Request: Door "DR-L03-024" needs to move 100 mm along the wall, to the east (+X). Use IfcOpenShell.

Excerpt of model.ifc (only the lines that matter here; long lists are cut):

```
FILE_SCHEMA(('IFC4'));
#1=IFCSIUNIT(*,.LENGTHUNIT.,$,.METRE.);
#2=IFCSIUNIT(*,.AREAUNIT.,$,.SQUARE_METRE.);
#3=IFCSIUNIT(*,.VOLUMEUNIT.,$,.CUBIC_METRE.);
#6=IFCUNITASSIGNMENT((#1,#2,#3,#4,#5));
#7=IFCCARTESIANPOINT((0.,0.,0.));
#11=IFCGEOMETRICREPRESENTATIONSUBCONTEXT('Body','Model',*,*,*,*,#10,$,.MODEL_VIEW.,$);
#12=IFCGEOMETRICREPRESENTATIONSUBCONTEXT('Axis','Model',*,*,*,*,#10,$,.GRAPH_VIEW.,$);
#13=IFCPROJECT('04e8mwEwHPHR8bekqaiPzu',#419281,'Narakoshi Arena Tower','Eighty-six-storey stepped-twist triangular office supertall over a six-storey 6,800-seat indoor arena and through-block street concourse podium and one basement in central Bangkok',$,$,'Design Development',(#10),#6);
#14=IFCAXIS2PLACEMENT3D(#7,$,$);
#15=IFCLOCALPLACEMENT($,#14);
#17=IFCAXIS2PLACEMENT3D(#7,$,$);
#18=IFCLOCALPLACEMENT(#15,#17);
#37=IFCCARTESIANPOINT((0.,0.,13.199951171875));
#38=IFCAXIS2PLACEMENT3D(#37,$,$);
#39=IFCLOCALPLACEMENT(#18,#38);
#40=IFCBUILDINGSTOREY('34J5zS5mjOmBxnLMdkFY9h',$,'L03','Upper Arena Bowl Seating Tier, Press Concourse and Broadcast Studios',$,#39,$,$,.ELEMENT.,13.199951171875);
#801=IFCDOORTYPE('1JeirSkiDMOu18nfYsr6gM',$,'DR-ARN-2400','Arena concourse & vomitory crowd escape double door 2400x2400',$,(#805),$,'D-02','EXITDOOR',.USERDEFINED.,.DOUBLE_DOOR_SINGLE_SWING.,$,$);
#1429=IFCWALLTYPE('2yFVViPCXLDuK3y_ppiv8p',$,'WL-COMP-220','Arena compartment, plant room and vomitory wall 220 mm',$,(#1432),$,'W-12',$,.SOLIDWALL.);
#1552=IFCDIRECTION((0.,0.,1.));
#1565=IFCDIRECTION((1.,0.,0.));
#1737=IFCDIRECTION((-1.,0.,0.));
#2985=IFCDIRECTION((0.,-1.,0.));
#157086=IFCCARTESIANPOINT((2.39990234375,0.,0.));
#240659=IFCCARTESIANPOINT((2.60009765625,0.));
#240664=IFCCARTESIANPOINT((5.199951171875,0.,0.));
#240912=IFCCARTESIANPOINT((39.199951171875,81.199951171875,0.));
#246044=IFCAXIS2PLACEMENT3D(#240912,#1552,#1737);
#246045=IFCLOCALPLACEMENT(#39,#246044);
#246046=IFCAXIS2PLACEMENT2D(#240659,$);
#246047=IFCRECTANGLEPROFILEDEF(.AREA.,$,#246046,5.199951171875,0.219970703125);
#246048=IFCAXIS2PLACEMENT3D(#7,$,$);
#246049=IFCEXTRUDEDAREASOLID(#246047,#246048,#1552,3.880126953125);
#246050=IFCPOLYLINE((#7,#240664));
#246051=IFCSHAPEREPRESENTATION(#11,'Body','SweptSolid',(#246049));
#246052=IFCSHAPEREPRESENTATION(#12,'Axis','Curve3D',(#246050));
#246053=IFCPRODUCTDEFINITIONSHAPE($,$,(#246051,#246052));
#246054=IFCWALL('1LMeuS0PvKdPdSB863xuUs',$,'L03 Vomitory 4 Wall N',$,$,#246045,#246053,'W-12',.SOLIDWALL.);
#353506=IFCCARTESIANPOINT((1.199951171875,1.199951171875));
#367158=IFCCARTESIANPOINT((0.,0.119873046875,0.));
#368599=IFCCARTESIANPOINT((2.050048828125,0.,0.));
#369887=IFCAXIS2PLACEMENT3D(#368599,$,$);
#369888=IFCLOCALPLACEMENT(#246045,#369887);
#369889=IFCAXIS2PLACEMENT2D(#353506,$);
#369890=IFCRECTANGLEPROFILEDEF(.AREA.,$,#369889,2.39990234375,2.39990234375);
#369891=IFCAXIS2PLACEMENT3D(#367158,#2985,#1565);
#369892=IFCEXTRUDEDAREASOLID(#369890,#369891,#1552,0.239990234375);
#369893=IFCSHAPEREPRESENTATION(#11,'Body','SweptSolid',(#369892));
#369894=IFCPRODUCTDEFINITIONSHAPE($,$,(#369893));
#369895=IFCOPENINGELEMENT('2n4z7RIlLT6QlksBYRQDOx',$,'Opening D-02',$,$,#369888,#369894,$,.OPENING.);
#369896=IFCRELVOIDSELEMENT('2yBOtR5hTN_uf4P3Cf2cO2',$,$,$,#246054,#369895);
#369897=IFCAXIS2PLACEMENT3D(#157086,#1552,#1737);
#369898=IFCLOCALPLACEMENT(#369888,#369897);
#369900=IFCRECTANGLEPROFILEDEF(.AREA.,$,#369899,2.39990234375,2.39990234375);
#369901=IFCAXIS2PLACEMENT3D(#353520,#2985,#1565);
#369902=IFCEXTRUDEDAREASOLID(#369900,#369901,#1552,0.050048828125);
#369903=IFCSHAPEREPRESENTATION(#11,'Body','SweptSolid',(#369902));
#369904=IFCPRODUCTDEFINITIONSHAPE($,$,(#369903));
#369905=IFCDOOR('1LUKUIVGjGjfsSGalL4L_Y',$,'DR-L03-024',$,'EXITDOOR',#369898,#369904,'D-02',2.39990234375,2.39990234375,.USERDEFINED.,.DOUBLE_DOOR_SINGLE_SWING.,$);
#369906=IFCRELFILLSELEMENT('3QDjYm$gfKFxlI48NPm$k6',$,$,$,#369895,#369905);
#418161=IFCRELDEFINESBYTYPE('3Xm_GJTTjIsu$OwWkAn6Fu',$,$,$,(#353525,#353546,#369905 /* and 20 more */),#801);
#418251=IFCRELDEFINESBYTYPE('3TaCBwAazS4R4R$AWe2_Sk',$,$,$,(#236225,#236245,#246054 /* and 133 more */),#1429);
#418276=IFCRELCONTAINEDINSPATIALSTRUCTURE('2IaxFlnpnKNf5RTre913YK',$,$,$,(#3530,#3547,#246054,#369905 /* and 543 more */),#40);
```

```python
import ifcopenshell
import ifcopenshell.api.geometry
import ifcopenshell.util.placement
import ifcopenshell.util.unit

model = ifcopenshell.open("model.ifc")
unit_scale = ifcopenshell.util.unit.calculate_unit_scale(model)

door = model.by_guid("1LUKUIVGjGjfsSGalL4L_Y")
opening = door.FillsVoids[0].RelatingOpeningElement
wall = opening.VoidsElements[0].RelatingBuildingElement

wall_matrix = ifcopenshell.util.placement.get_local_placement(wall.ObjectPlacement)
shift = wall_matrix[:3, 0] * -0.1 / unit_scale
before = ifcopenshell.util.placement.get_local_placement(door.ObjectPlacement)[:3, 3].copy()

# The door is placed relative to its opening, so it follows when the opening moves.
matrix = ifcopenshell.util.placement.get_local_placement(opening.ObjectPlacement)
matrix[:3, 3] += shift
ifcopenshell.api.geometry.edit_object_placement(
    model, product=opening, matrix=matrix, is_si=False, should_transform_children=True
)

after = ifcopenshell.util.placement.get_local_placement(door.ObjectPlacement)[:3, 3]
print("door moved by", (after - before).round(3) + 0.0)

model.write("model_updated.ifc")
```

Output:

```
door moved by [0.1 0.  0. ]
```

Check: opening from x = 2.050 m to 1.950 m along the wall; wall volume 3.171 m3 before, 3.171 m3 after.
